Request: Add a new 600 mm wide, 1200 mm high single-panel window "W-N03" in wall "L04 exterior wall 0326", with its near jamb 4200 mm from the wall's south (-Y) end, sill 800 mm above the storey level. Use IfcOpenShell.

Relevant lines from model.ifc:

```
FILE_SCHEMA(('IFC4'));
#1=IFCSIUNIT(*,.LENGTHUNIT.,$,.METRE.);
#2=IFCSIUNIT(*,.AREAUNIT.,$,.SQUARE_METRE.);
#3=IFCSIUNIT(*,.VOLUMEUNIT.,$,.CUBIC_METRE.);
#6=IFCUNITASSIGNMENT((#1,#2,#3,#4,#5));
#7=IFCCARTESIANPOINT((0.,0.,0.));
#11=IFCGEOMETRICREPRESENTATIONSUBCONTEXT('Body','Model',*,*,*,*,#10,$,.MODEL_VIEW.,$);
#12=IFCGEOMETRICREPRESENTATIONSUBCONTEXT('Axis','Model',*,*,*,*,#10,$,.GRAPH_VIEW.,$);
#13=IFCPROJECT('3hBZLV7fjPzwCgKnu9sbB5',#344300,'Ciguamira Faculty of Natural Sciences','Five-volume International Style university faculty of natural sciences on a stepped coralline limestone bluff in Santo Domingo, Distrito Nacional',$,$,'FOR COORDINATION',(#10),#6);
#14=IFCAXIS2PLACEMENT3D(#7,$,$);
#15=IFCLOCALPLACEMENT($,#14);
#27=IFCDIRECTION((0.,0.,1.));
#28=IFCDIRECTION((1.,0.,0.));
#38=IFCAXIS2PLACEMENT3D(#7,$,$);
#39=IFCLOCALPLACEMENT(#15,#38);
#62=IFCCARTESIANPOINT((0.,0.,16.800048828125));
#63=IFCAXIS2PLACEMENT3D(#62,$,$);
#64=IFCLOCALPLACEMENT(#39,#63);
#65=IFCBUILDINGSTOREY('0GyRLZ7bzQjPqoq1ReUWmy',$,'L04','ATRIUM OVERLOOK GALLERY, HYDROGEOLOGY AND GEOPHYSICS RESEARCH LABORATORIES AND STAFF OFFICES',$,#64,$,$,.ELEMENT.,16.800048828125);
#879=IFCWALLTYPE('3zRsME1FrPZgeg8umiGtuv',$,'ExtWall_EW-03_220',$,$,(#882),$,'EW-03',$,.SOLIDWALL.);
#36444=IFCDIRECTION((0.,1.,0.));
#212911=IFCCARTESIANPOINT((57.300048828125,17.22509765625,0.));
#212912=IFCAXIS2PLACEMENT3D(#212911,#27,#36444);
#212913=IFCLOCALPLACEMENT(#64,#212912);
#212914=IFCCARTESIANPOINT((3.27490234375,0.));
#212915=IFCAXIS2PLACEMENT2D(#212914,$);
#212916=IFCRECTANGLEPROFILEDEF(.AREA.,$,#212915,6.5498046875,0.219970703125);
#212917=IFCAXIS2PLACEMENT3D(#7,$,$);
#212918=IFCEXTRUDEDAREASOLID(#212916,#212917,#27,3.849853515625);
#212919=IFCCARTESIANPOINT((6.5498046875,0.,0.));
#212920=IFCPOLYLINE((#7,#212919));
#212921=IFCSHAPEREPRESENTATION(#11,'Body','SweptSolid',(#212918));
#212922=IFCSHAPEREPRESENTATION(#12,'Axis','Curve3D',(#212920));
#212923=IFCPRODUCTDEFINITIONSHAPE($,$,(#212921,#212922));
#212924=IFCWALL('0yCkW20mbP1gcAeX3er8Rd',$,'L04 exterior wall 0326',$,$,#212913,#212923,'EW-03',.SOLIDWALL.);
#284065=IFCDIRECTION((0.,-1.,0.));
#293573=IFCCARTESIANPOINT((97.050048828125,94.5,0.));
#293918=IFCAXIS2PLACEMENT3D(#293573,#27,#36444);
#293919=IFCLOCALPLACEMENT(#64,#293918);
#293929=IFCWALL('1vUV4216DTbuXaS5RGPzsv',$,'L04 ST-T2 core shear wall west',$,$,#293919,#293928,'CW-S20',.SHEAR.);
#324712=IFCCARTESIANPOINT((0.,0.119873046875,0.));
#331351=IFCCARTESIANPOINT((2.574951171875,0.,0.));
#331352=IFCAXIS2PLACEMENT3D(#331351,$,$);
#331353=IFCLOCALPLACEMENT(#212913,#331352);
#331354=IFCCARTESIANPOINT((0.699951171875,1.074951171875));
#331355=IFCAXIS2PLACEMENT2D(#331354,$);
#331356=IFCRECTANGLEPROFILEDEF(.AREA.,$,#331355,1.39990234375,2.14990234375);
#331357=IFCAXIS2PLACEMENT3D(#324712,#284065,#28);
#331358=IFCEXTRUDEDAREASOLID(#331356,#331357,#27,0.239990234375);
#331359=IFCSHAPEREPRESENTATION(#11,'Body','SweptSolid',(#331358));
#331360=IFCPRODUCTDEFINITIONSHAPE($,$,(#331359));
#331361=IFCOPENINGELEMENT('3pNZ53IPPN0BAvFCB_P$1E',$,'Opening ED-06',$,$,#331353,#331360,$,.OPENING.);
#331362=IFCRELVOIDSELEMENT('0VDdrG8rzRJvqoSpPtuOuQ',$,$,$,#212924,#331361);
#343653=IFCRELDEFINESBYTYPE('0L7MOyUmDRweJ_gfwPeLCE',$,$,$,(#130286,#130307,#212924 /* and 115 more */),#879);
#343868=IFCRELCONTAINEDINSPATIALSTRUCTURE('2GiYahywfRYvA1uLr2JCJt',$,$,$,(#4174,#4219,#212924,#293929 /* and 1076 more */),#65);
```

```python
import numpy as np
import ifcopenshell
import ifcopenshell.api.feature
import ifcopenshell.api.geometry
import ifcopenshell.api.root
import ifcopenshell.api.spatial
import ifcopenshell.geom
import ifcopenshell.util.element
import ifcopenshell.util.placement
import ifcopenshell.util.representation
import ifcopenshell.util.shape
import ifcopenshell.util.unit

model = ifcopenshell.open("model.ifc")
unit_scale = ifcopenshell.util.unit.calculate_unit_scale(model)
settings = ifcopenshell.geom.settings()


def volume(element):
    """Net volume in cubic metres, openings subtracted."""
    shape = ifcopenshell.geom.create_shape(settings, element)
    return ifcopenshell.util.shape.get_volume(shape.geometry)


wall = model.by_guid("0yCkW20mbP1gcAeX3er8Rd")
storey = ifcopenshell.util.element.get_container(wall, ifc_class="IfcBuildingStorey")
context = ifcopenshell.util.representation.get_context(model, "Model", "Body", "MODEL_VIEW")
before = volume(wall)

width, height, from_end, sill = 0.6, 1.2, 4.2, 0.8  # metres

# The wall runs along its own X axis, and the end named is its -X end.
wall_shape = ifcopenshell.geom.create_shape(settings, wall)
x, y, z = ifcopenshell.util.shape.get_vertices(wall_shape.geometry).T
start = x.min() + from_end
face, thickness = float(y.min()), float(y.max() - y.min())
wall_matrix = ifcopenshell.util.placement.get_local_placement(wall.ObjectPlacement)
level = ifcopenshell.util.placement.get_local_placement(storey.ObjectPlacement)[2, 3]


def in_wall(x, y):
    """Placement at x, y metres in the wall's axes, at sill height."""
    matrix = wall_matrix.copy()
    matrix[:, 3] = wall_matrix @ np.array([x / unit_scale, y / unit_scale, 0.0, 1.0])
    matrix[2, 3] = level + sill / unit_scale
    return matrix


# Opening: a box that overshoots both wall faces by 50 mm.
opening = ifcopenshell.api.root.create_entity(model, ifc_class="IfcOpeningElement", predefined_type="OPENING")
box = ifcopenshell.api.geometry.add_wall_representation(
    model, context=context, length=width, height=height, thickness=thickness + 0.1
)
ifcopenshell.api.geometry.assign_representation(model, product=opening, representation=box)
ifcopenshell.api.geometry.edit_object_placement(model, product=opening, matrix=in_wall(start, face - 0.05), is_si=False)
ifcopenshell.api.feature.add_feature(model, feature=opening, element=wall)

window = ifcopenshell.api.root.create_entity(model, ifc_class="IfcWindow", name="W-N03", predefined_type="WINDOW")
window.OverallWidth, window.OverallHeight = width / unit_scale, height / unit_scale
window.PartitioningType = "SINGLE_PANEL"
body = ifcopenshell.api.geometry.add_window_representation(
    model,
    context=context,
    overall_width=window.OverallWidth,
    overall_height=window.OverallHeight,
    partition_type="SINGLE_PANEL",
)
ifcopenshell.api.geometry.assign_representation(model, product=window, representation=body)
ifcopenshell.api.spatial.assign_container(model, products=[window], relating_structure=storey)
ifcopenshell.api.feature.add_filling(model, opening=opening, element=window)

# Centre the window in the wall's thickness.
ifcopenshell.api.geometry.edit_object_placement(model, product=window, matrix=in_wall(start, face), is_si=False)
window_shape = ifcopenshell.geom.create_shape(settings, window)
depth = ifcopenshell.util.shape.get_vertices(window_shape.geometry)[:, 1]
offset = face + thickness / 2 - (depth.min() + depth.max()) / 2
ifcopenshell.api.geometry.edit_object_placement(model, product=window, matrix=in_wall(start, offset), is_si=False)

after = volume(wall)

print(f"wall volume {before:.3f} -> {after:.3f} m3")

model.write("model-out.ifc")
```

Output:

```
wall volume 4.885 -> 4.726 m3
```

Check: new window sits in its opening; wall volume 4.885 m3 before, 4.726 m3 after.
